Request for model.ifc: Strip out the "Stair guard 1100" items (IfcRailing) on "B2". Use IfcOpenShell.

First a look at what the model holds.

```python
import ifcopenshell
import ifcopenshell.util.element

model = ifcopenshell.open("model.ifc")
print(model.schema)
storey = next(s for s in model.by_type("IfcBuildingStorey") if s.Name == "B2")
railings = [e for e in ifcopenshell.util.element.get_decomposition(storey) if e.is_a("IfcRailing")]
seen = {}
for e in railings:
    element_type = ifcopenshell.util.element.get_type(e)
    name = element_type.Name if element_type not in (None, e) else None
    seen[name] = seen.get(name, 0) + 1
for name, count in sorted(seen.items(), key=str):
    print(count, "x", name)
```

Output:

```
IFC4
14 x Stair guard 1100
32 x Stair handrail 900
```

```python
import ifcopenshell
import ifcopenshell.api.root
import ifcopenshell.util.element

model = ifcopenshell.open("model.ifc")

storey = next(s for s in model.by_type("IfcBuildingStorey") if s.Name == "B2")
railings = [e for e in ifcopenshell.util.element.get_decomposition(storey) if e.is_a("IfcRailing")]
targets = [e for e in railings if (t := ifcopenshell.util.element.get_type(e)) not in (None, e) and t.Name == "Stair guard 1100"]

for e in targets:
    ifcopenshell.api.root.remove_product(model, product=e)
print(len(targets), "removed")

model.write("model-out.ifc")
```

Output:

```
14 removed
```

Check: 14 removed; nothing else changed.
